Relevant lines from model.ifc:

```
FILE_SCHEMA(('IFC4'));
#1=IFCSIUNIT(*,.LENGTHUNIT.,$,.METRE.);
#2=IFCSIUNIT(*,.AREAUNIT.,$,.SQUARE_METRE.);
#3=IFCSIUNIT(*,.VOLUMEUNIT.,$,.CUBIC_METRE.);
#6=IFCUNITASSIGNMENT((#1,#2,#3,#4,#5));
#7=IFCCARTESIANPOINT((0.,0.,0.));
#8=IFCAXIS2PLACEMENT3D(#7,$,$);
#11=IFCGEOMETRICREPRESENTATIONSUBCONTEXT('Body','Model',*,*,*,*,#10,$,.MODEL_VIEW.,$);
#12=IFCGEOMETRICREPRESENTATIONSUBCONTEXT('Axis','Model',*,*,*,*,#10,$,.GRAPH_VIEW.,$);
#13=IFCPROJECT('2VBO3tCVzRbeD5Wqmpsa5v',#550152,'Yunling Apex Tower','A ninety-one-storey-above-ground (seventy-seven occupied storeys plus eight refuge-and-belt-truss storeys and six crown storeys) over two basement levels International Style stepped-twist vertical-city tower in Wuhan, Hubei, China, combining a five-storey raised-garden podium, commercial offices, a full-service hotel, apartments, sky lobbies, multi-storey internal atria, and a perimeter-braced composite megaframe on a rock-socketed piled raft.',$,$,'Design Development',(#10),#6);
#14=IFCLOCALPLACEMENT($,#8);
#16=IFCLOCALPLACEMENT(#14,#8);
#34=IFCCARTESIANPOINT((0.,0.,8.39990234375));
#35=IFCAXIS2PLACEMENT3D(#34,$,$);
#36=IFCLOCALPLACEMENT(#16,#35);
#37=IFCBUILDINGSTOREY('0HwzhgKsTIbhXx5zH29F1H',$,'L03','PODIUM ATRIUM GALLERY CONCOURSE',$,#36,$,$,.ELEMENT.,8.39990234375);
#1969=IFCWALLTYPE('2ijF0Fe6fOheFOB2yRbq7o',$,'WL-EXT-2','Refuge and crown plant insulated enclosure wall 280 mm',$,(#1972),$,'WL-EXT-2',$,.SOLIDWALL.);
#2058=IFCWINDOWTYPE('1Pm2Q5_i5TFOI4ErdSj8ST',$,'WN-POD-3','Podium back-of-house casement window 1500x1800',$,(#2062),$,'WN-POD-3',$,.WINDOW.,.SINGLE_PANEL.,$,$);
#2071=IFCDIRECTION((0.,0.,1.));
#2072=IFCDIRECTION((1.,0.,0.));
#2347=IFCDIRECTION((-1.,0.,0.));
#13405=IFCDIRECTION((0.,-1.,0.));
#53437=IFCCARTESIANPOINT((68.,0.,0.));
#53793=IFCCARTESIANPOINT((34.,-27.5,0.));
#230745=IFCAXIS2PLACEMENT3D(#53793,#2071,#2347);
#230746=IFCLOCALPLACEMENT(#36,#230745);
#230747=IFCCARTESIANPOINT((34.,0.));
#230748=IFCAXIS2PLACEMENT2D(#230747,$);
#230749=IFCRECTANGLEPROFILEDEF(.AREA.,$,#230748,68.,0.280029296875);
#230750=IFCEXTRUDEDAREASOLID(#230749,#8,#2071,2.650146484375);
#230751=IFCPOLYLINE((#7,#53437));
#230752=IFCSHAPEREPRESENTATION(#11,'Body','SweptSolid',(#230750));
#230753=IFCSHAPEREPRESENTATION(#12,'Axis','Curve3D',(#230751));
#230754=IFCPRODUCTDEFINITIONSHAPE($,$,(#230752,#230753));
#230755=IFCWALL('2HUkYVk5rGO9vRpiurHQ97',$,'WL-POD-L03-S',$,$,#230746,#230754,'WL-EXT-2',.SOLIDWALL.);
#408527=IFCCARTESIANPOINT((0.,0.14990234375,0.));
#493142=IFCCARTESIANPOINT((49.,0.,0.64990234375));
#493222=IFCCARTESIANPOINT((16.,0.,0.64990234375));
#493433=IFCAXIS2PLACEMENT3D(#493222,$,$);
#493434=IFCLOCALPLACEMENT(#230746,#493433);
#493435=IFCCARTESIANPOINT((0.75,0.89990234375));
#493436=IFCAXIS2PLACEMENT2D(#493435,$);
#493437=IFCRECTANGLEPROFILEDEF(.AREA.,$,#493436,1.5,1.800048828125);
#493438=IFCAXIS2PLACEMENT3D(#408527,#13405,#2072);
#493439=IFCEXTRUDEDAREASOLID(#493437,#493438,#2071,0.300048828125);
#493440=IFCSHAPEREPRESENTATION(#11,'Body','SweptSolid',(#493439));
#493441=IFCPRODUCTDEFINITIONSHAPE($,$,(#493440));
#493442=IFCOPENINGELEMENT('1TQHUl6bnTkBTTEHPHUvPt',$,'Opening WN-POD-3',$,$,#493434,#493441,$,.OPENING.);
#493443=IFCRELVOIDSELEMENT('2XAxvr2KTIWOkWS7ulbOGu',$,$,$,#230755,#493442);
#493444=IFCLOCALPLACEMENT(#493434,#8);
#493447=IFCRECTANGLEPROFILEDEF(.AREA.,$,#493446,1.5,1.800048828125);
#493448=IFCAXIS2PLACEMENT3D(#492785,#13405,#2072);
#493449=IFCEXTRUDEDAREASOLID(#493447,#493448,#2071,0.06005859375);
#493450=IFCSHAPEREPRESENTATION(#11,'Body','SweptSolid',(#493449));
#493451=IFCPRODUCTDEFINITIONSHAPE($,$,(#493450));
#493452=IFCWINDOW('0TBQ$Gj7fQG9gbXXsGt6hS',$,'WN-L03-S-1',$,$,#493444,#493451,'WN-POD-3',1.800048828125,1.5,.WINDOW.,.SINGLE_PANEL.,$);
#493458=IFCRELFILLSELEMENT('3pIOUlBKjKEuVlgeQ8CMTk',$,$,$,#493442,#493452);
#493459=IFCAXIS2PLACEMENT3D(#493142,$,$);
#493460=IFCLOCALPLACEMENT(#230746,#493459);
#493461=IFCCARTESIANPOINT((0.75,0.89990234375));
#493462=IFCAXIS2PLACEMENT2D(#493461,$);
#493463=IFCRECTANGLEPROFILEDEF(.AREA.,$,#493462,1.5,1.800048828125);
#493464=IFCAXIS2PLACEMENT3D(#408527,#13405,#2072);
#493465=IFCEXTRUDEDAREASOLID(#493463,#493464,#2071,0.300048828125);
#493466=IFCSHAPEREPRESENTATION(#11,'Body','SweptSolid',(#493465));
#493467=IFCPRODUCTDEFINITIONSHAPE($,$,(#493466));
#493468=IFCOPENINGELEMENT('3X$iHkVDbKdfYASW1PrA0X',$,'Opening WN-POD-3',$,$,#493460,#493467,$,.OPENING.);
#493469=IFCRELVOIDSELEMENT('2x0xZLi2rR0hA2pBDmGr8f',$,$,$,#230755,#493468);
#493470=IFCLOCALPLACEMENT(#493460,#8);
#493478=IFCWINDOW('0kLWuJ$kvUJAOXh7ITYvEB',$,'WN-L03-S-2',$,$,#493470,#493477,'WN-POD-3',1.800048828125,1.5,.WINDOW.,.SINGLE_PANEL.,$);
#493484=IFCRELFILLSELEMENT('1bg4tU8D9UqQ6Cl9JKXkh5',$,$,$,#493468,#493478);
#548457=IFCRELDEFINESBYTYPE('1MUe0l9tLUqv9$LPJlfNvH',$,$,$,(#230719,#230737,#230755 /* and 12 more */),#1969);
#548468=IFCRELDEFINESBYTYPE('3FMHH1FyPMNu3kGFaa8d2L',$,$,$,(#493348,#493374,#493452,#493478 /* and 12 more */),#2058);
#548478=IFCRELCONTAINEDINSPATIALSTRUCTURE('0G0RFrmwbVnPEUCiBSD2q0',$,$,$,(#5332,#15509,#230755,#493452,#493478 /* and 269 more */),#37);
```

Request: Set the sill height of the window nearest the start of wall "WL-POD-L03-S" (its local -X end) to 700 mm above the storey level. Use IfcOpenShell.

```python
import numpy as np
import ifcopenshell
import ifcopenshell.api.geometry
import ifcopenshell.geom
import ifcopenshell.util.element
import ifcopenshell.util.placement
import ifcopenshell.util.shape
import ifcopenshell.util.unit

model = ifcopenshell.open("model.ifc")
unit_scale = ifcopenshell.util.unit.calculate_unit_scale(model)

window = model.by_guid("0TBQ$Gj7fQG9gbXXsGt6hS")
opening = window.FillsVoids[0].RelatingOpeningElement
storey = ifcopenshell.util.element.get_container(window, ifc_class="IfcBuildingStorey")
level = ifcopenshell.util.placement.get_local_placement(storey.ObjectPlacement)[2, 3]

# The opening's origin need not be at the sill, so measure its lowest point.
shape = ifcopenshell.geom.create_shape(ifcopenshell.geom.settings(), opening)
bottom = ifcopenshell.util.shape.get_shape_bottom_elevation(shape, shape.geometry) / unit_scale
dz = level + 0.7 / unit_scale - bottom

shift = np.array([0.0, 0.0, dz])
# The window is placed relative to its opening, so it follows when the opening moves.
matrix = ifcopenshell.util.placement.get_local_placement(opening.ObjectPlacement)
matrix[:3, 3] += shift
ifcopenshell.api.geometry.edit_object_placement(
    model, product=opening, matrix=matrix, is_si=False, should_transform_children=True
)

print(f"moved by {dz * unit_scale:+.3f} m")

model.write("model_edited.ifc")
```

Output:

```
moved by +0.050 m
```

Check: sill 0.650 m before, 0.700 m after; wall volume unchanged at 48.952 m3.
